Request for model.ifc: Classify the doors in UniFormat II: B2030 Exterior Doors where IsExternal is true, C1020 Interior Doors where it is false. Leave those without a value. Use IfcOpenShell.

First a look at what the model holds.

```python
import ifcopenshell
import ifcopenshell.util.element

model = ifcopenshell.open("model.ifc")
print(model.schema)
print("classifications:", [c.Name for c in model.by_type("IfcClassification")])
values = [ifcopenshell.util.element.get_pset(e, "Pset_DoorCommon", "IsExternal") for e in model.by_type("IfcDoor")]
for value in (True, False, None):
    print("IsExternal", value, values.count(value))
```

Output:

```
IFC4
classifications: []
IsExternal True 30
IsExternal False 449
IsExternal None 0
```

```python
import ifcopenshell
import ifcopenshell.api.classification
import ifcopenshell.util.element

model = ifcopenshell.open("model.ifc")

system = ifcopenshell.api.classification.add_classification(model, classification="UniFormat II")

doors = model.by_type("IfcDoor")
external = {e: ifcopenshell.util.element.get_pset(e, "Pset_DoorCommon", "IsExternal") for e in doors}
for flag, code, name in ((True, "B2030", "Exterior Doors"), (False, "C1020", "Interior Doors")):
    products = [e for e in doors if external[e] is flag]
    ifcopenshell.api.classification.add_reference(
        model, products=products, classification=system, identification=code, name=name
    )
    print(code, len(products))

model.write("model_edited.ifc")
```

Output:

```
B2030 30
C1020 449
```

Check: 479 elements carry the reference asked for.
